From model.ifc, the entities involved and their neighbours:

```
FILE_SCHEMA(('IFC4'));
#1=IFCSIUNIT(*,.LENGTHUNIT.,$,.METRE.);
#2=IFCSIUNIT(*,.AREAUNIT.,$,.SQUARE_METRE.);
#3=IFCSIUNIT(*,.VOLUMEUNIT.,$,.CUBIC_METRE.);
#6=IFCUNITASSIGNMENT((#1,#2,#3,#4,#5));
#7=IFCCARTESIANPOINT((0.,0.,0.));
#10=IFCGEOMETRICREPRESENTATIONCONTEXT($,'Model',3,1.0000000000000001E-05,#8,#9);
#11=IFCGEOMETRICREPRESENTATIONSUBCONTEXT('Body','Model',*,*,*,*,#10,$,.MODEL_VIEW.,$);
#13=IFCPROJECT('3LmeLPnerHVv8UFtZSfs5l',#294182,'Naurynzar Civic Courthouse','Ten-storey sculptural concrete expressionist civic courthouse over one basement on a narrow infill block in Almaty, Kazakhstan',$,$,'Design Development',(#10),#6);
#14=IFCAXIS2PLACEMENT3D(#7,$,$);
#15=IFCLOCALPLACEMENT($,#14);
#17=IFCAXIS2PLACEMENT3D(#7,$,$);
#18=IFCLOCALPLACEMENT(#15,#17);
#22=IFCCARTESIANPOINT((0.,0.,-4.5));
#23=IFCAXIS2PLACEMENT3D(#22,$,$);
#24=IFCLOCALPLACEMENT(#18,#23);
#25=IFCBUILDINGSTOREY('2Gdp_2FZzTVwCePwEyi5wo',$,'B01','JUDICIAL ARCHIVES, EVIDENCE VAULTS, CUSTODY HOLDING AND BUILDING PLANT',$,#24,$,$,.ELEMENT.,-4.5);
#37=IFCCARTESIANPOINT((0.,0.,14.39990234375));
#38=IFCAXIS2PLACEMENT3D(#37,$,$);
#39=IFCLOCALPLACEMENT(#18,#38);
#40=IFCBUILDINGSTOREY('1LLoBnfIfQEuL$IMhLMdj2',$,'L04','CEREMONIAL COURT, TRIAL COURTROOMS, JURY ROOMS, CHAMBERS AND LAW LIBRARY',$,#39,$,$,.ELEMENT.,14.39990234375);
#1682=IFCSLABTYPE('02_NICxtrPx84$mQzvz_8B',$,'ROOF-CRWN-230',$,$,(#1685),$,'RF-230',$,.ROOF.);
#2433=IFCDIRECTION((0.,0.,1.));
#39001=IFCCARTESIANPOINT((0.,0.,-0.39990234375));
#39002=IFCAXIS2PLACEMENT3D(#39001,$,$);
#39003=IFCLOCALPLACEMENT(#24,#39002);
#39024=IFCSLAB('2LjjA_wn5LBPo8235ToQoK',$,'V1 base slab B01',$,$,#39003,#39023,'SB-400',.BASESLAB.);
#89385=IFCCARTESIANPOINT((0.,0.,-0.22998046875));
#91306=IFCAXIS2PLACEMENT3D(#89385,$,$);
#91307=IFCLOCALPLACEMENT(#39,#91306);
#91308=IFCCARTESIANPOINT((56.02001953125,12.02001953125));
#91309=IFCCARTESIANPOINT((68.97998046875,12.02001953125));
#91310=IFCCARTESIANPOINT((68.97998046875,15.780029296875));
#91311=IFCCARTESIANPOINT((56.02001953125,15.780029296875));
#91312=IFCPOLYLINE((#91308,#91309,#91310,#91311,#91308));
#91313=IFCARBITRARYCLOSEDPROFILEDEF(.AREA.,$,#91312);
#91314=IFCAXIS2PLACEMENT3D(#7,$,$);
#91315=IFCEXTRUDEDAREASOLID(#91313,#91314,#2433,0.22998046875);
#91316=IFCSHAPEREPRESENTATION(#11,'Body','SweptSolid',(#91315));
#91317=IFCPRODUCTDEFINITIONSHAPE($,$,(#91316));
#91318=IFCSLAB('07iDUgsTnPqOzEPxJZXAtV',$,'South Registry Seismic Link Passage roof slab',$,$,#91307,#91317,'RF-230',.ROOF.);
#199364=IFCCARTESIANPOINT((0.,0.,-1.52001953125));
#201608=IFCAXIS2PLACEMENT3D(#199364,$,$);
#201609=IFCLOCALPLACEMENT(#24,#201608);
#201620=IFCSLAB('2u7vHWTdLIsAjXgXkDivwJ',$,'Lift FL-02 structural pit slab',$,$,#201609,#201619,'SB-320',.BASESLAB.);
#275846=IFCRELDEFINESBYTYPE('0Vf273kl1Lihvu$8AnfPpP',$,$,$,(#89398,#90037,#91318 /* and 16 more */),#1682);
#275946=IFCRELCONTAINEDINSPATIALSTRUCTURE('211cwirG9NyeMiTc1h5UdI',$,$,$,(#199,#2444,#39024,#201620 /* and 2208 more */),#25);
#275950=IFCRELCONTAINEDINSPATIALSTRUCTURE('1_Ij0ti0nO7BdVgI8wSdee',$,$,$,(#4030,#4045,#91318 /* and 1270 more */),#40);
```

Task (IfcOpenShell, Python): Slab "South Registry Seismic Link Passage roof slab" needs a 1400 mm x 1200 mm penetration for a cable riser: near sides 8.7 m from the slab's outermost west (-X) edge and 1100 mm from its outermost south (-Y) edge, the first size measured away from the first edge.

```python
import numpy as np
import ifcopenshell
import ifcopenshell.api.feature
import ifcopenshell.api.geometry
import ifcopenshell.api.root
import ifcopenshell.geom
import ifcopenshell.util.placement
import ifcopenshell.util.representation
import ifcopenshell.util.shape
import ifcopenshell.util.unit

model = ifcopenshell.open("model.ifc")
unit_scale = ifcopenshell.util.unit.calculate_unit_scale(model)
settings = ifcopenshell.geom.settings()


def volume(element):
    """Net volume in cubic metres, openings subtracted."""
    shape = ifcopenshell.geom.create_shape(settings, element)
    return ifcopenshell.util.shape.get_volume(shape.geometry)


slab = model.by_id(91318)
before = volume(slab)

# Extent in the slab's own axes, in metres. The edges named are its -X and -Y sides.
slab_shape = ifcopenshell.geom.create_shape(settings, slab)
vertices = ifcopenshell.util.shape.get_vertices(slab_shape.geometry)
x_min, y_min, bottom = vertices.min(axis=0)
top = vertices[:, 2].max()

opening = ifcopenshell.api.root.create_entity(model, ifc_class="IfcOpeningElement", name="Cable riser opening", predefined_type="OPENING")
context = ifcopenshell.util.representation.get_context(model, "Model", "Body", "MODEL_VIEW")
width, depth = 1.4, 1.2
outline = [(0.0, 0.0), (width, 0.0), (width, depth), (0.0, depth), (0.0, 0.0)]
# Overshoot both faces by 50 mm so the cut is clean.
shape = ifcopenshell.api.geometry.add_slab_representation(
    model, context=context, depth=top - bottom + 0.1, polyline=outline
)
ifcopenshell.api.geometry.assign_representation(model, product=opening, representation=shape)

matrix = ifcopenshell.util.placement.get_local_placement(slab.ObjectPlacement)
matrix[:, 3] = matrix @ np.append(np.array([x_min + 8.7, y_min + 1.1, bottom - 0.05]) / unit_scale, 1.0)
ifcopenshell.api.geometry.edit_object_placement(model, product=opening, matrix=matrix, is_si=False)
ifcopenshell.api.feature.add_feature(model, feature=opening, element=slab)

after = volume(slab)

print(f"slab volume {before:.3f} -> {after:.3f} m3")

model.write("model_rev.ifc")
```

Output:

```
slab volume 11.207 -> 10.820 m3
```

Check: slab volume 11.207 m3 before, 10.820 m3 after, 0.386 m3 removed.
